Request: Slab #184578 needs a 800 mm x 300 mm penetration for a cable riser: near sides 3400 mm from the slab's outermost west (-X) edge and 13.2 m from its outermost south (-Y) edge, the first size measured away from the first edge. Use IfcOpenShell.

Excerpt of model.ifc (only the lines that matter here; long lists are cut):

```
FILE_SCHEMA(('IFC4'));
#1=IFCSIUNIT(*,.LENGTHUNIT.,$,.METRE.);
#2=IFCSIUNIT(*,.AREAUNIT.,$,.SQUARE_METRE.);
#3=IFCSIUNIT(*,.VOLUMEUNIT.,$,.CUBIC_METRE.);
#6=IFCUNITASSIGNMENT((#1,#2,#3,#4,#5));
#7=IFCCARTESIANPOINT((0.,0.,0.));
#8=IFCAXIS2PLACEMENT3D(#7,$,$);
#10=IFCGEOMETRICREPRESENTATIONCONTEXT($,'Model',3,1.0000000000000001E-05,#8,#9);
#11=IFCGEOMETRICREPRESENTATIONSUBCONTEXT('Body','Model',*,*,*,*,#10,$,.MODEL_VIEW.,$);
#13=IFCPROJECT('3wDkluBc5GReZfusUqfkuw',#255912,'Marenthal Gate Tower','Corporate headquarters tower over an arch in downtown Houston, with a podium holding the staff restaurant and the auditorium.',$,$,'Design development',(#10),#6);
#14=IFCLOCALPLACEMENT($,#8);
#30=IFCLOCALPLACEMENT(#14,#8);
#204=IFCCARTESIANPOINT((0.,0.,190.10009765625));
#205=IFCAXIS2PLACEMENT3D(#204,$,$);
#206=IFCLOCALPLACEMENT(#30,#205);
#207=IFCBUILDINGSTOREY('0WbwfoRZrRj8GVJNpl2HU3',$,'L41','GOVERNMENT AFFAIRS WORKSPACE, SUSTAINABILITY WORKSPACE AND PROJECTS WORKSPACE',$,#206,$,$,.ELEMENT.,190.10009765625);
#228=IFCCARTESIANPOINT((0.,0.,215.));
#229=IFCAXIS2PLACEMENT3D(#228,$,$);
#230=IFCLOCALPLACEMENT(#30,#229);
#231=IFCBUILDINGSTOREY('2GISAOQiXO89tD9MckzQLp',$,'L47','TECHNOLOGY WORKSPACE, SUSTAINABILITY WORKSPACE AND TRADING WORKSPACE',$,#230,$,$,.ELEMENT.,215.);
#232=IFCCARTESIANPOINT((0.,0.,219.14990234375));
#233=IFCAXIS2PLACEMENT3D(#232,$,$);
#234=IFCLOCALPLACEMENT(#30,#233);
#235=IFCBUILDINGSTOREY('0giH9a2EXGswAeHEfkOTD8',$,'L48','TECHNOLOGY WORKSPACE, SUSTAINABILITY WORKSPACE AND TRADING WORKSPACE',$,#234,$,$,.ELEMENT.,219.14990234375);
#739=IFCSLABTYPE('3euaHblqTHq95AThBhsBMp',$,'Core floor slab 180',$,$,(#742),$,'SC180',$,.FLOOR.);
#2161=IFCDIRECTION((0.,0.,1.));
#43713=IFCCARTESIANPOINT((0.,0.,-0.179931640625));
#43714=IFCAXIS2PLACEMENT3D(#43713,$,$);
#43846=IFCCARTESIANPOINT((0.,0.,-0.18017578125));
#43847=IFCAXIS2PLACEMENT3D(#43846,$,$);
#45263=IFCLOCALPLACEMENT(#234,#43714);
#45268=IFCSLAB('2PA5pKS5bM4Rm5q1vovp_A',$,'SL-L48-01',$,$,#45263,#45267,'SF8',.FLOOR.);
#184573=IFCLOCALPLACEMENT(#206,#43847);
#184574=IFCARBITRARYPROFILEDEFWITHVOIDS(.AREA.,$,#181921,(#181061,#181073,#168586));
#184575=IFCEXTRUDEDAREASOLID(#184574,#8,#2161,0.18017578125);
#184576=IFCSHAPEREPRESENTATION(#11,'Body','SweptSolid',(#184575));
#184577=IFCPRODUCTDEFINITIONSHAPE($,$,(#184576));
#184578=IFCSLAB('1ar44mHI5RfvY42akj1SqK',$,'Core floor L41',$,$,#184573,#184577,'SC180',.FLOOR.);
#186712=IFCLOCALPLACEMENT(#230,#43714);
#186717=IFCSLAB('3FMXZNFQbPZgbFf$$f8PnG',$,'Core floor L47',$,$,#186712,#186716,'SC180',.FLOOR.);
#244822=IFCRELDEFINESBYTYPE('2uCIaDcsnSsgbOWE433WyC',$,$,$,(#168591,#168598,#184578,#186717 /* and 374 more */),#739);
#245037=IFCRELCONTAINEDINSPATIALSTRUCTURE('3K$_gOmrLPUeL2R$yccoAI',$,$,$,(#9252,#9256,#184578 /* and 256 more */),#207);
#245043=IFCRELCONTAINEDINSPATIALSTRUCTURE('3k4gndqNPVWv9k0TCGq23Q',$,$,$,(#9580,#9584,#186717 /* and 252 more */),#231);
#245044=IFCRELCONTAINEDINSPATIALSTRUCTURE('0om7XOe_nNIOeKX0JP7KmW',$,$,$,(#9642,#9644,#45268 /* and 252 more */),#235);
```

```python
import numpy as np
import ifcopenshell
import ifcopenshell.api.feature
import ifcopenshell.api.geometry
import ifcopenshell.api.root
import ifcopenshell.geom
import ifcopenshell.util.placement
import ifcopenshell.util.representation
import ifcopenshell.util.shape
import ifcopenshell.util.unit

model = ifcopenshell.open("model.ifc")
unit_scale = ifcopenshell.util.unit.calculate_unit_scale(model)
settings = ifcopenshell.geom.settings()


def volume(element):
    """Net volume in cubic metres, openings subtracted."""
    shape = ifcopenshell.geom.create_shape(settings, element)
    return ifcopenshell.util.shape.get_volume(shape.geometry)


slab = model.by_guid("1ar44mHI5RfvY42akj1SqK")
before = volume(slab)

# Extent in the slab's own axes, in metres. The edges named are its -X and -Y sides.
slab_shape = ifcopenshell.geom.create_shape(settings, slab)
vertices = ifcopenshell.util.shape.get_vertices(slab_shape.geometry)
x_min, y_min, bottom = vertices.min(axis=0)
top = vertices[:, 2].max()

opening = ifcopenshell.api.root.create_entity(model, ifc_class="IfcOpeningElement", name="Cable riser opening", predefined_type="OPENING")
context = ifcopenshell.util.representation.get_context(model, "Model", "Body", "MODEL_VIEW")
width, depth = 0.8, 0.3
outline = [(0.0, 0.0), (width, 0.0), (width, depth), (0.0, depth), (0.0, 0.0)]
# Overshoot both faces by 50 mm so the cut is clean.
shape = ifcopenshell.api.geometry.add_slab_representation(
    model, context=context, depth=top - bottom + 0.1, polyline=outline
)
ifcopenshell.api.geometry.assign_representation(model, product=opening, representation=shape)

matrix = ifcopenshell.util.placement.get_local_placement(slab.ObjectPlacement)
matrix[:, 3] = matrix @ np.append(np.array([x_min + 3.4, y_min + 13.2, bottom - 0.05]) / unit_scale, 1.0)
ifcopenshell.api.geometry.edit_object_placement(model, product=opening, matrix=matrix, is_si=False)
ifcopenshell.api.feature.add_feature(model, feature=opening, element=slab)

after = volume(slab)

print(f"slab volume {before:.3f} -> {after:.3f} m3")

model.write("model_updated.ifc")
```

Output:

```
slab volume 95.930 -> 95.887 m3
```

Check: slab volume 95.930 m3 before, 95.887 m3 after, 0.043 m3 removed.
